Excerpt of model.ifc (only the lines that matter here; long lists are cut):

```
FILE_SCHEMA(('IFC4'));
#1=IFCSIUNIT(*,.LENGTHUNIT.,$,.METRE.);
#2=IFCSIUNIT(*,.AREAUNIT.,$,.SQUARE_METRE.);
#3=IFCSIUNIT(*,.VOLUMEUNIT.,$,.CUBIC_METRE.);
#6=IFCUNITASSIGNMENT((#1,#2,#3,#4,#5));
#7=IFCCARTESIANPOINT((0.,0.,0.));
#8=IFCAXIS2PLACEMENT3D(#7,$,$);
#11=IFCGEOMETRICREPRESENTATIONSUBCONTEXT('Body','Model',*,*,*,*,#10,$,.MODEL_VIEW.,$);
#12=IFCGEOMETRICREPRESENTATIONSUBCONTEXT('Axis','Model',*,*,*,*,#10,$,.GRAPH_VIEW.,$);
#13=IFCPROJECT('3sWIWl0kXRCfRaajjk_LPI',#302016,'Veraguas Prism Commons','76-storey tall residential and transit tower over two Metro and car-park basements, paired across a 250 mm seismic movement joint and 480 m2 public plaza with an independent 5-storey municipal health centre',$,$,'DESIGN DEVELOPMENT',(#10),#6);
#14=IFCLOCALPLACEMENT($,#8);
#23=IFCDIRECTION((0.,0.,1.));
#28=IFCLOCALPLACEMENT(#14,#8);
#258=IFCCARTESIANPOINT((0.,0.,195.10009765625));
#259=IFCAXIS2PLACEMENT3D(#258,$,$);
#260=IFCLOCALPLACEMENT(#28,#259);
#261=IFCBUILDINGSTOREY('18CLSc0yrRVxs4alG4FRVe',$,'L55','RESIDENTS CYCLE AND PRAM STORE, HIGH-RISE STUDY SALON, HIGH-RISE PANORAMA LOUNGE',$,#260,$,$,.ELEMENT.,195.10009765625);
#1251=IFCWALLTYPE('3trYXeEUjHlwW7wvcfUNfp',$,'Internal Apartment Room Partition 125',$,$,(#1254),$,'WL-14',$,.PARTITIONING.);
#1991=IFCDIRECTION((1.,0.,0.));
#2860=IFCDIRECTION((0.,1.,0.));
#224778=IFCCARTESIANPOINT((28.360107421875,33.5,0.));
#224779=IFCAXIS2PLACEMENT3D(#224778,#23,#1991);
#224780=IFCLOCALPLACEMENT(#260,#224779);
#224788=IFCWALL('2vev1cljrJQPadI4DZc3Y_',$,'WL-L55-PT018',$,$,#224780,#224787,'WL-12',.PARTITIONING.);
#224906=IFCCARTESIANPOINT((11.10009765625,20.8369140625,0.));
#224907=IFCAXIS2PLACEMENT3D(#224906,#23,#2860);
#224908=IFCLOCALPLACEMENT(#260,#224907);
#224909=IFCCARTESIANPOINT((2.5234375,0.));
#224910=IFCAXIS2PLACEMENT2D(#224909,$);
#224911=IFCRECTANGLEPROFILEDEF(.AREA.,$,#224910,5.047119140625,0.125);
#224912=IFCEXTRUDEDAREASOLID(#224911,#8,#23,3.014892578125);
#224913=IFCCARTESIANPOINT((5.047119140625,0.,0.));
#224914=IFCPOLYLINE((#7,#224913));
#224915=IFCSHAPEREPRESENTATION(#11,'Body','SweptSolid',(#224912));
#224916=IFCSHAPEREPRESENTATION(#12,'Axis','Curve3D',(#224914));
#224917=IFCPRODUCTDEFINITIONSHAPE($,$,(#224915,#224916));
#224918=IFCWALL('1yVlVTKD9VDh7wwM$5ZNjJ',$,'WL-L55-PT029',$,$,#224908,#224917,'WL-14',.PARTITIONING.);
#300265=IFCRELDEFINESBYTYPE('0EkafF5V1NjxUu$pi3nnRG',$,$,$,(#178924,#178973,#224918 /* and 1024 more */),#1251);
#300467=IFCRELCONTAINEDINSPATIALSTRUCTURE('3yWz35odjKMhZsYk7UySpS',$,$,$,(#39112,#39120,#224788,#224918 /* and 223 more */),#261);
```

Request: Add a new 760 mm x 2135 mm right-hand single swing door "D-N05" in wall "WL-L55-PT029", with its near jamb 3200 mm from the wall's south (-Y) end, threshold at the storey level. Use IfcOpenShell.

```python
import numpy as np
import ifcopenshell
import ifcopenshell.api.feature
import ifcopenshell.api.geometry
import ifcopenshell.api.root
import ifcopenshell.api.spatial
import ifcopenshell.geom
import ifcopenshell.util.element
import ifcopenshell.util.placement
import ifcopenshell.util.representation
import ifcopenshell.util.shape
import ifcopenshell.util.unit

model = ifcopenshell.open("model.ifc")
unit_scale = ifcopenshell.util.unit.calculate_unit_scale(model)
settings = ifcopenshell.geom.settings()


def volume(element):
    """Net volume in cubic metres, openings subtracted."""
    shape = ifcopenshell.geom.create_shape(settings, element)
    return ifcopenshell.util.shape.get_volume(shape.geometry)


wall = model.by_guid("1yVlVTKD9VDh7wwM$5ZNjJ")
storey = ifcopenshell.util.element.get_container(wall, ifc_class="IfcBuildingStorey")
context = ifcopenshell.util.representation.get_context(model, "Model", "Body", "MODEL_VIEW")
before = volume(wall)

width, height, from_end, sill = 0.76, 2.135, 3.2, 0.0  # metres

# The wall runs along its own X axis, and the end named is its -X end.
wall_shape = ifcopenshell.geom.create_shape(settings, wall)
x, y, z = ifcopenshell.util.shape.get_vertices(wall_shape.geometry).T
start = x.min() + from_end
face, thickness = float(y.min()), float(y.max() - y.min())
wall_matrix = ifcopenshell.util.placement.get_local_placement(wall.ObjectPlacement)
level = ifcopenshell.util.placement.get_local_placement(storey.ObjectPlacement)[2, 3]


def in_wall(x, y):
    """Placement at x, y metres in the wall's axes, at sill height."""
    matrix = wall_matrix.copy()
    matrix[:, 3] = wall_matrix @ np.array([x / unit_scale, y / unit_scale, 0.0, 1.0])
    matrix[2, 3] = level + sill / unit_scale
    return matrix


# Opening: a box that overshoots both wall faces by 50 mm.
opening = ifcopenshell.api.root.create_entity(model, ifc_class="IfcOpeningElement", predefined_type="OPENING")
box = ifcopenshell.api.geometry.add_wall_representation(
    model, context=context, length=width, height=height, thickness=thickness + 0.1
)
ifcopenshell.api.geometry.assign_representation(model, product=opening, representation=box)
ifcopenshell.api.geometry.edit_object_placement(model, product=opening, matrix=in_wall(start, face - 0.05), is_si=False)
ifcopenshell.api.feature.add_feature(model, feature=opening, element=wall)

door = ifcopenshell.api.root.create_entity(model, ifc_class="IfcDoor", name="D-N05", predefined_type="DOOR")
door.OverallWidth, door.OverallHeight = width / unit_scale, height / unit_scale
door.OperationType = "SINGLE_SWING_RIGHT"
body = ifcopenshell.api.geometry.add_door_representation(
    model,
    context=context,
    overall_width=door.OverallWidth,
    overall_height=door.OverallHeight,
    operation_type="SINGLE_SWING_RIGHT",
    lining_properties={"LiningDepth": thickness / unit_scale, "ThresholdDepth": thickness / unit_scale},
)
ifcopenshell.api.geometry.assign_representation(model, product=door, representation=body)
ifcopenshell.api.spatial.assign_container(model, products=[door], relating_structure=storey)
ifcopenshell.api.feature.add_filling(model, opening=opening, element=door)

# The lining spans the wall, so the door starts at the wall face.
ifcopenshell.api.geometry.edit_object_placement(model, product=door, matrix=in_wall(start, face), is_si=False)

after = volume(wall)

print(f"wall volume {before:.3f} -> {after:.3f} m3")

model.write("model_rev.ifc")
```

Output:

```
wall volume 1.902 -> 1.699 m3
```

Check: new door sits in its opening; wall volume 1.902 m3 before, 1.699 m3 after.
